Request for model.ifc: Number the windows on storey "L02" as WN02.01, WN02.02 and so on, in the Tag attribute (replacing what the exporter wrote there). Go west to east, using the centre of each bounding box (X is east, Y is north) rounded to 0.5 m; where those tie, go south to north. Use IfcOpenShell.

First a look at what the model holds.

```python
import ifcopenshell
import ifcopenshell.util.element
import ifcopenshell.util.placement

model = ifcopenshell.open("model.ifc")
print(model.schema)
storey = next(s for s in model.by_type("IfcBuildingStorey") if s.Name == "L02")
windows = [e for e in ifcopenshell.util.element.get_decomposition(storey) if e.is_a("IfcWindow")]
for e in sorted(windows, key=lambda e: e.id()):
    origin = ifcopenshell.util.placement.get_local_placement(e.ObjectPlacement)[:3, 3]
    print(e.id(), e.Tag, e.Name, origin.round(2) + 0.0, sep=" | ")
```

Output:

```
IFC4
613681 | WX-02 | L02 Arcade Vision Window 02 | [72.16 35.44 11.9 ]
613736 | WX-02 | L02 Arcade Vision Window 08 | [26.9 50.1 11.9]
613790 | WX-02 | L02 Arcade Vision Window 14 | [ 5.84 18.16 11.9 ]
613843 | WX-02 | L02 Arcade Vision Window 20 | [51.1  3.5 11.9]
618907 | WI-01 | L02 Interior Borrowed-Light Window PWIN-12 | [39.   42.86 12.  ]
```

```python
import ifcopenshell
import ifcopenshell.geom
import ifcopenshell.util.element
import ifcopenshell.util.shape

model = ifcopenshell.open("model.ifc")
settings = ifcopenshell.geom.settings()
settings.set("use-world-coords", True)


def centre(element):
    shape = ifcopenshell.geom.create_shape(settings, element)
    return ifcopenshell.util.shape.get_bbox_centroid(shape.geometry)


storey = next(s for s in model.by_type("IfcBuildingStorey") if s.Name == "L02")
windows = [e for e in ifcopenshell.util.element.get_decomposition(storey) if e.is_a("IfcWindow")]

# Insertion points can sit at a corner or the storey origin, so sort by the geometry (in metres).
centres = {e: centre(e) for e in windows}
windows.sort(key=lambda e: (round(centres[e][0] / 0.5), centres[e][1]))

for i, e in enumerate(windows, start=1):
    number = f"WN02.{i:02d}"
    e.Tag = number
    print(e.id(), number)

model.write("model_rev.ifc")
```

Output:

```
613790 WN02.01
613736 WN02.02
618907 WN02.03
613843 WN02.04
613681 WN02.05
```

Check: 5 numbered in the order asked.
